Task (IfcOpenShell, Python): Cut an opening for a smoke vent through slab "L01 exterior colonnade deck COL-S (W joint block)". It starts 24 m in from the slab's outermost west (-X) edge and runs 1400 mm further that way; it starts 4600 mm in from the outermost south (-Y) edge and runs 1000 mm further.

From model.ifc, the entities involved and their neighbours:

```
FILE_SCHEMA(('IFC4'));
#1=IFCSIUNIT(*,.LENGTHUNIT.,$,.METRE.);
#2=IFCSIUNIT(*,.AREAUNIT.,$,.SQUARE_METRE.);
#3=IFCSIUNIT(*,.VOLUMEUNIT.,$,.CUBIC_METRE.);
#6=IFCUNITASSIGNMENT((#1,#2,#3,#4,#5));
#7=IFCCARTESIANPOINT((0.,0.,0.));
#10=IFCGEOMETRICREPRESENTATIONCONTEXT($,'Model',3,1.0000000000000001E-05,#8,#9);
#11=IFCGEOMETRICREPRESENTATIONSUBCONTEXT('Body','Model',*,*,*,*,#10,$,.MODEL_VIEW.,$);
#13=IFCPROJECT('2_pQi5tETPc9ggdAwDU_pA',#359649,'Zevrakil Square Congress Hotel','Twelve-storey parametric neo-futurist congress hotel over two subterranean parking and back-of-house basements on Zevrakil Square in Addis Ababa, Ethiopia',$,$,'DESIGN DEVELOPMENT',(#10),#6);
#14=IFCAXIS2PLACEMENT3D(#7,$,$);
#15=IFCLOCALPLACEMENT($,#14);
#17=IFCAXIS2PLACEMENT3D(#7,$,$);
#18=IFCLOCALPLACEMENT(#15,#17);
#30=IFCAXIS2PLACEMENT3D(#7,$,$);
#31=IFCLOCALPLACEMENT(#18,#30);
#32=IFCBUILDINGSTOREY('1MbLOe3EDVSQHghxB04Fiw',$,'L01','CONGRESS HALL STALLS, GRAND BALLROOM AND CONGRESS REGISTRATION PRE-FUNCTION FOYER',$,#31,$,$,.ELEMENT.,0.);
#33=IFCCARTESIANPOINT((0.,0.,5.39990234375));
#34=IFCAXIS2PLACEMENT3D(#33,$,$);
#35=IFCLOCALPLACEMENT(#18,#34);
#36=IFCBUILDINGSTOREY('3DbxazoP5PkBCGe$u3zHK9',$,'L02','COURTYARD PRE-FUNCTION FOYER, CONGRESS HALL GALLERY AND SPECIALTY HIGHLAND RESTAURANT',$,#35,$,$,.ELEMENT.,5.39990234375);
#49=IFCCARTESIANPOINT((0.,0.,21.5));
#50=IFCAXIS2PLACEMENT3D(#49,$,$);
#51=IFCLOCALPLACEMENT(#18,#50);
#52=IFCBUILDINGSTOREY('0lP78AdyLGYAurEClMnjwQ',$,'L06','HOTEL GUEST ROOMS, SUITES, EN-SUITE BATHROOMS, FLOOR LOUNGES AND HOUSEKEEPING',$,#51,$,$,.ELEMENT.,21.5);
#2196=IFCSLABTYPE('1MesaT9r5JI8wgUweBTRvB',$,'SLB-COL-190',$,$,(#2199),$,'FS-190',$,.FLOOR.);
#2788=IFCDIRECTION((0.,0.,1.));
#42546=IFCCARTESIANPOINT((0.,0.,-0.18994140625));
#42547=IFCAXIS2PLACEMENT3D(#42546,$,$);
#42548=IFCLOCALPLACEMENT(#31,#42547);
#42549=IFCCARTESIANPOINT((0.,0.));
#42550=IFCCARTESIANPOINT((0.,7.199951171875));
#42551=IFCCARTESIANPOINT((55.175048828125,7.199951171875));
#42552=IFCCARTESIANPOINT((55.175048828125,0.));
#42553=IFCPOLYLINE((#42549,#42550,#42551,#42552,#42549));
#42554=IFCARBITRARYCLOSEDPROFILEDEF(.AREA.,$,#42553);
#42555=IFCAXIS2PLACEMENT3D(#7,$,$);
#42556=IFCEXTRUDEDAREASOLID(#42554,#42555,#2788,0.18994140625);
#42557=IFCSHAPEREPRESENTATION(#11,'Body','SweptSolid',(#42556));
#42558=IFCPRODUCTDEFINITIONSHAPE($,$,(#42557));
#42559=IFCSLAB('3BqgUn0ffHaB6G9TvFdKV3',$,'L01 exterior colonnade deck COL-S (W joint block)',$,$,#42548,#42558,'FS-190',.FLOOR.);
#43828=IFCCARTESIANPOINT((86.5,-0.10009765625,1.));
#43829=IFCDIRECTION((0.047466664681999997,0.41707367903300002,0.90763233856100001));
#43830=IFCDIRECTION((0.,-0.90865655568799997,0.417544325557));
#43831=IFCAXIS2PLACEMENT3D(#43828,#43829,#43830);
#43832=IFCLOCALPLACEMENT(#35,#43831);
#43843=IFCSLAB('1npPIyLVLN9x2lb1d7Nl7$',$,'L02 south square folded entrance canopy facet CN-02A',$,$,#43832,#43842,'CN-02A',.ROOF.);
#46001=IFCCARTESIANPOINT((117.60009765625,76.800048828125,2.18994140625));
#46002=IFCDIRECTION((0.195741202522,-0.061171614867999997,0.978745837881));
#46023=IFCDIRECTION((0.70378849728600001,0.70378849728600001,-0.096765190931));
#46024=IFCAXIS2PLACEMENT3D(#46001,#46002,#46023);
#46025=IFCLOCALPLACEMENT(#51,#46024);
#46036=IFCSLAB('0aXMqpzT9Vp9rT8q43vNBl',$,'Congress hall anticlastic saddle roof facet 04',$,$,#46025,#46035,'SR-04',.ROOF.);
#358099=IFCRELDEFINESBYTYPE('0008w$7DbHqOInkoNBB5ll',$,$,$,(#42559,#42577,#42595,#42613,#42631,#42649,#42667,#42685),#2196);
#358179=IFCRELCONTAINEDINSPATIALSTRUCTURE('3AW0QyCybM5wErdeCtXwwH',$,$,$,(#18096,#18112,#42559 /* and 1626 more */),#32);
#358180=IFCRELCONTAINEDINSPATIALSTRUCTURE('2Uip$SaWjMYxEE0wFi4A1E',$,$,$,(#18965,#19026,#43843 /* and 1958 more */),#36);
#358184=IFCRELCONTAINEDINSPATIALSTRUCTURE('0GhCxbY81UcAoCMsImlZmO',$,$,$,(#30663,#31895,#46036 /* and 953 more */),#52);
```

```python
import numpy as np
import ifcopenshell
import ifcopenshell.api.feature
import ifcopenshell.api.geometry
import ifcopenshell.api.root
import ifcopenshell.geom
import ifcopenshell.util.placement
import ifcopenshell.util.representation
import ifcopenshell.util.shape
import ifcopenshell.util.unit

model = ifcopenshell.open("model.ifc")
unit_scale = ifcopenshell.util.unit.calculate_unit_scale(model)
settings = ifcopenshell.geom.settings()


def volume(element):
    """Net volume in cubic metres, openings subtracted."""
    shape = ifcopenshell.geom.create_shape(settings, element)
    return ifcopenshell.util.shape.get_volume(shape.geometry)


slab = model.by_guid("3BqgUn0ffHaB6G9TvFdKV3")
before = volume(slab)

# Extent in the slab's own axes, in metres. The edges named are its -X and -Y sides.
slab_shape = ifcopenshell.geom.create_shape(settings, slab)
vertices = ifcopenshell.util.shape.get_vertices(slab_shape.geometry)
x_min, y_min, bottom = vertices.min(axis=0)
top = vertices[:, 2].max()

opening = ifcopenshell.api.root.create_entity(model, ifc_class="IfcOpeningElement", name="Smoke vent opening", predefined_type="OPENING")
context = ifcopenshell.util.representation.get_context(model, "Model", "Body", "MODEL_VIEW")
width, depth = 1.4, 1
outline = [(0.0, 0.0), (width, 0.0), (width, depth), (0.0, depth), (0.0, 0.0)]
# Overshoot both faces by 50 mm so the cut is clean.
shape = ifcopenshell.api.geometry.add_slab_representation(
    model, context=context, depth=top - bottom + 0.1, polyline=outline
)
ifcopenshell.api.geometry.assign_representation(model, product=opening, representation=shape)

matrix = ifcopenshell.util.placement.get_local_placement(slab.ObjectPlacement)
matrix[:, 3] = matrix @ np.append(np.array([x_min + 24, y_min + 4.6, bottom - 0.05]) / unit_scale, 1.0)
ifcopenshell.api.geometry.edit_object_placement(model, product=opening, matrix=matrix, is_si=False)
ifcopenshell.api.feature.add_feature(model, feature=opening, element=slab)

after = volume(slab)

print(f"slab volume {before:.3f} -> {after:.3f} m3")

model.write("model_rev.ifc")
```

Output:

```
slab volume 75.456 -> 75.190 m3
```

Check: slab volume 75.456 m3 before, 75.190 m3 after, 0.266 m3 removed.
